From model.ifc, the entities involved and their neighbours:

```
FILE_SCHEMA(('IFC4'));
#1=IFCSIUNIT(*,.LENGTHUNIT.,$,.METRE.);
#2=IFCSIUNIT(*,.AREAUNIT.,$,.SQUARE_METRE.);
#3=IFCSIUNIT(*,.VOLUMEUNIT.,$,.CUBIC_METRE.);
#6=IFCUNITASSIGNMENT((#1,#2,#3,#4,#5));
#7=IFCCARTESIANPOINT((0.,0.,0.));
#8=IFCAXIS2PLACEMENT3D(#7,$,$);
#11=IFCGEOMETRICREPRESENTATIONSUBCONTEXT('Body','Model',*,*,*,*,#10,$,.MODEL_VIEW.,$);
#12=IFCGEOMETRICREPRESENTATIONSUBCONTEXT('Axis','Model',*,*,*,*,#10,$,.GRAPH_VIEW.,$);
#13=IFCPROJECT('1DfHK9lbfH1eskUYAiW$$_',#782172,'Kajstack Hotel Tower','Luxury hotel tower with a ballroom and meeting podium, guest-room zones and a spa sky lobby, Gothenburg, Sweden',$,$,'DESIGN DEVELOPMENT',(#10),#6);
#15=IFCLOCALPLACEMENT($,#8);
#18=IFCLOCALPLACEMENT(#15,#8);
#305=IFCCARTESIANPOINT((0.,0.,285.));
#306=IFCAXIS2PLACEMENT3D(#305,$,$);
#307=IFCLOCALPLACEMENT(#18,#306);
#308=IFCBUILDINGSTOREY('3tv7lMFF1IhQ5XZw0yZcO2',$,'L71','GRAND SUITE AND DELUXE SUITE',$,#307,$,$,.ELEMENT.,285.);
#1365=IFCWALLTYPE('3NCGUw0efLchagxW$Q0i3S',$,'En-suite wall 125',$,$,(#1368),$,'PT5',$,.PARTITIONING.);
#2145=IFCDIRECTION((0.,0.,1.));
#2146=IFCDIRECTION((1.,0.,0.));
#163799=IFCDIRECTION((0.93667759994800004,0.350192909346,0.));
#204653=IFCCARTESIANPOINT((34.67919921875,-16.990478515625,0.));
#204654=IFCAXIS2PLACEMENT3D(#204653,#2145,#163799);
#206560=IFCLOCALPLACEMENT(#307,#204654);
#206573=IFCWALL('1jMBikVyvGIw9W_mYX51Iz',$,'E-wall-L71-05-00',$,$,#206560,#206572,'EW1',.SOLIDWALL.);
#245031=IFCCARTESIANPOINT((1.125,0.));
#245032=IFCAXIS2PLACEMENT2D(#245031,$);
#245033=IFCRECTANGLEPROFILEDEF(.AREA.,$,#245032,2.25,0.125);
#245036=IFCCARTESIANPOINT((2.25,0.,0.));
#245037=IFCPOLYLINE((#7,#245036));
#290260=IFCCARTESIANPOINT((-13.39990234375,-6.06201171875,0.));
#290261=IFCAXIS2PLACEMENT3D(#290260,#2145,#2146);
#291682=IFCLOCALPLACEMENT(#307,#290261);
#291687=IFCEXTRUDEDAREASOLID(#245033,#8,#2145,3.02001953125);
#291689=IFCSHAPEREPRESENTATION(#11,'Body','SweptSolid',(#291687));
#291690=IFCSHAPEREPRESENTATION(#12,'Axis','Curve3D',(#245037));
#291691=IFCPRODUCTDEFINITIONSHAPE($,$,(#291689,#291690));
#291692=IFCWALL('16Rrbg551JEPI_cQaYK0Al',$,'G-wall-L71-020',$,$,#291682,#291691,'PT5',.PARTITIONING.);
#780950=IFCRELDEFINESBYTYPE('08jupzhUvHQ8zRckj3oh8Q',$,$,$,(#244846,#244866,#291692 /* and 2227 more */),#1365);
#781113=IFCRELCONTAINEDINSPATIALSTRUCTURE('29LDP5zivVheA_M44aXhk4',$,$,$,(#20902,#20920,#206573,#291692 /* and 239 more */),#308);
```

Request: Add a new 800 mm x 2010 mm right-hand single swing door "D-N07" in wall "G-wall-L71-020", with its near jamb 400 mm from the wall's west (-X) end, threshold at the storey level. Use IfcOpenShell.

```python
import numpy as np
import ifcopenshell
import ifcopenshell.api.feature
import ifcopenshell.api.geometry
import ifcopenshell.api.root
import ifcopenshell.api.spatial
import ifcopenshell.geom
import ifcopenshell.util.element
import ifcopenshell.util.placement
import ifcopenshell.util.representation
import ifcopenshell.util.shape
import ifcopenshell.util.unit

model = ifcopenshell.open("model.ifc")
unit_scale = ifcopenshell.util.unit.calculate_unit_scale(model)
settings = ifcopenshell.geom.settings()


def volume(element):
    """Net volume in cubic metres, openings subtracted."""
    shape = ifcopenshell.geom.create_shape(settings, element)
    return ifcopenshell.util.shape.get_volume(shape.geometry)


wall = model.by_guid("16Rrbg551JEPI_cQaYK0Al")
storey = ifcopenshell.util.element.get_container(wall, ifc_class="IfcBuildingStorey")
context = ifcopenshell.util.representation.get_context(model, "Model", "Body", "MODEL_VIEW")
before = volume(wall)

width, height, from_end, sill = 0.8, 2.01, 0.4, 0.0  # metres

# The wall runs along its own X axis, and the end named is its -X end.
wall_shape = ifcopenshell.geom.create_shape(settings, wall)
x, y, z = ifcopenshell.util.shape.get_vertices(wall_shape.geometry).T
start = x.min() + from_end
face, thickness = float(y.min()), float(y.max() - y.min())
wall_matrix = ifcopenshell.util.placement.get_local_placement(wall.ObjectPlacement)
level = ifcopenshell.util.placement.get_local_placement(storey.ObjectPlacement)[2, 3]


def in_wall(x, y):
    """Placement at x, y metres in the wall's axes, at sill height."""
    matrix = wall_matrix.copy()
    matrix[:, 3] = wall_matrix @ np.array([x / unit_scale, y / unit_scale, 0.0, 1.0])
    matrix[2, 3] = level + sill / unit_scale
    return matrix


# Opening: a box that overshoots both wall faces by 50 mm.
opening = ifcopenshell.api.root.create_entity(model, ifc_class="IfcOpeningElement", predefined_type="OPENING")
box = ifcopenshell.api.geometry.add_wall_representation(
    model, context=context, length=width, height=height, thickness=thickness + 0.1
)
ifcopenshell.api.geometry.assign_representation(model, product=opening, representation=box)
ifcopenshell.api.geometry.edit_object_placement(model, product=opening, matrix=in_wall(start, face - 0.05), is_si=False)
ifcopenshell.api.feature.add_feature(model, feature=opening, element=wall)

door = ifcopenshell.api.root.create_entity(model, ifc_class="IfcDoor", name="D-N07", predefined_type="DOOR")
door.OverallWidth, door.OverallHeight = width / unit_scale, height / unit_scale
door.OperationType = "SINGLE_SWING_RIGHT"
body = ifcopenshell.api.geometry.add_door_representation(
    model,
    context=context,
    overall_width=door.OverallWidth,
    overall_height=door.OverallHeight,
    operation_type="SINGLE_SWING_RIGHT",
    lining_properties={"LiningDepth": thickness / unit_scale, "ThresholdDepth": thickness / unit_scale},
)
ifcopenshell.api.geometry.assign_representation(model, product=door, representation=body)
ifcopenshell.api.spatial.assign_container(model, products=[door], relating_structure=storey)
ifcopenshell.api.feature.add_filling(model, opening=opening, element=door)

# The lining spans the wall, so the door starts at the wall face.
ifcopenshell.api.geometry.edit_object_placement(model, product=door, matrix=in_wall(start, face), is_si=False)

after = volume(wall)

print(f"wall volume {before:.3f} -> {after:.3f} m3")

model.write("model_updated.ifc")
```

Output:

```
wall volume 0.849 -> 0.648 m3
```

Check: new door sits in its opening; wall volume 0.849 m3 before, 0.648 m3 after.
